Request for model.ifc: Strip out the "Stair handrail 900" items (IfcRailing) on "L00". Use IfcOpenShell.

First a look at what the model holds.

```python
import ifcopenshell
import ifcopenshell.util.element

model = ifcopenshell.open("model.ifc")
print(model.schema)
storey = next(s for s in model.by_type("IfcBuildingStorey") if s.Name == "L00")
railings = [e for e in ifcopenshell.util.element.get_decomposition(storey) if e.is_a("IfcRailing")]
seen = {}
for e in railings:
    element_type = ifcopenshell.util.element.get_type(e)
    name = element_type.Name if element_type not in (None, e) else None
    seen[name] = seen.get(name, 0) + 1
for name, count in sorted(seen.items(), key=str):
    print(count, "x", name)
```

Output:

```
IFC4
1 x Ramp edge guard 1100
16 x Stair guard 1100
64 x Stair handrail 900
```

```python
import ifcopenshell
import ifcopenshell.api.root
import ifcopenshell.util.element

model = ifcopenshell.open("model.ifc")

storey = next(s for s in model.by_type("IfcBuildingStorey") if s.Name == "L00")
railings = [e for e in ifcopenshell.util.element.get_decomposition(storey) if e.is_a("IfcRailing")]
targets = [e for e in railings if (t := ifcopenshell.util.element.get_type(e)) not in (None, e) and t.Name == "Stair handrail 900"]

for e in targets:
    ifcopenshell.api.root.remove_product(model, product=e)
print(len(targets), "removed")

model.write("model_v2.ifc")
```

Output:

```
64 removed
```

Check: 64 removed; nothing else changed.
